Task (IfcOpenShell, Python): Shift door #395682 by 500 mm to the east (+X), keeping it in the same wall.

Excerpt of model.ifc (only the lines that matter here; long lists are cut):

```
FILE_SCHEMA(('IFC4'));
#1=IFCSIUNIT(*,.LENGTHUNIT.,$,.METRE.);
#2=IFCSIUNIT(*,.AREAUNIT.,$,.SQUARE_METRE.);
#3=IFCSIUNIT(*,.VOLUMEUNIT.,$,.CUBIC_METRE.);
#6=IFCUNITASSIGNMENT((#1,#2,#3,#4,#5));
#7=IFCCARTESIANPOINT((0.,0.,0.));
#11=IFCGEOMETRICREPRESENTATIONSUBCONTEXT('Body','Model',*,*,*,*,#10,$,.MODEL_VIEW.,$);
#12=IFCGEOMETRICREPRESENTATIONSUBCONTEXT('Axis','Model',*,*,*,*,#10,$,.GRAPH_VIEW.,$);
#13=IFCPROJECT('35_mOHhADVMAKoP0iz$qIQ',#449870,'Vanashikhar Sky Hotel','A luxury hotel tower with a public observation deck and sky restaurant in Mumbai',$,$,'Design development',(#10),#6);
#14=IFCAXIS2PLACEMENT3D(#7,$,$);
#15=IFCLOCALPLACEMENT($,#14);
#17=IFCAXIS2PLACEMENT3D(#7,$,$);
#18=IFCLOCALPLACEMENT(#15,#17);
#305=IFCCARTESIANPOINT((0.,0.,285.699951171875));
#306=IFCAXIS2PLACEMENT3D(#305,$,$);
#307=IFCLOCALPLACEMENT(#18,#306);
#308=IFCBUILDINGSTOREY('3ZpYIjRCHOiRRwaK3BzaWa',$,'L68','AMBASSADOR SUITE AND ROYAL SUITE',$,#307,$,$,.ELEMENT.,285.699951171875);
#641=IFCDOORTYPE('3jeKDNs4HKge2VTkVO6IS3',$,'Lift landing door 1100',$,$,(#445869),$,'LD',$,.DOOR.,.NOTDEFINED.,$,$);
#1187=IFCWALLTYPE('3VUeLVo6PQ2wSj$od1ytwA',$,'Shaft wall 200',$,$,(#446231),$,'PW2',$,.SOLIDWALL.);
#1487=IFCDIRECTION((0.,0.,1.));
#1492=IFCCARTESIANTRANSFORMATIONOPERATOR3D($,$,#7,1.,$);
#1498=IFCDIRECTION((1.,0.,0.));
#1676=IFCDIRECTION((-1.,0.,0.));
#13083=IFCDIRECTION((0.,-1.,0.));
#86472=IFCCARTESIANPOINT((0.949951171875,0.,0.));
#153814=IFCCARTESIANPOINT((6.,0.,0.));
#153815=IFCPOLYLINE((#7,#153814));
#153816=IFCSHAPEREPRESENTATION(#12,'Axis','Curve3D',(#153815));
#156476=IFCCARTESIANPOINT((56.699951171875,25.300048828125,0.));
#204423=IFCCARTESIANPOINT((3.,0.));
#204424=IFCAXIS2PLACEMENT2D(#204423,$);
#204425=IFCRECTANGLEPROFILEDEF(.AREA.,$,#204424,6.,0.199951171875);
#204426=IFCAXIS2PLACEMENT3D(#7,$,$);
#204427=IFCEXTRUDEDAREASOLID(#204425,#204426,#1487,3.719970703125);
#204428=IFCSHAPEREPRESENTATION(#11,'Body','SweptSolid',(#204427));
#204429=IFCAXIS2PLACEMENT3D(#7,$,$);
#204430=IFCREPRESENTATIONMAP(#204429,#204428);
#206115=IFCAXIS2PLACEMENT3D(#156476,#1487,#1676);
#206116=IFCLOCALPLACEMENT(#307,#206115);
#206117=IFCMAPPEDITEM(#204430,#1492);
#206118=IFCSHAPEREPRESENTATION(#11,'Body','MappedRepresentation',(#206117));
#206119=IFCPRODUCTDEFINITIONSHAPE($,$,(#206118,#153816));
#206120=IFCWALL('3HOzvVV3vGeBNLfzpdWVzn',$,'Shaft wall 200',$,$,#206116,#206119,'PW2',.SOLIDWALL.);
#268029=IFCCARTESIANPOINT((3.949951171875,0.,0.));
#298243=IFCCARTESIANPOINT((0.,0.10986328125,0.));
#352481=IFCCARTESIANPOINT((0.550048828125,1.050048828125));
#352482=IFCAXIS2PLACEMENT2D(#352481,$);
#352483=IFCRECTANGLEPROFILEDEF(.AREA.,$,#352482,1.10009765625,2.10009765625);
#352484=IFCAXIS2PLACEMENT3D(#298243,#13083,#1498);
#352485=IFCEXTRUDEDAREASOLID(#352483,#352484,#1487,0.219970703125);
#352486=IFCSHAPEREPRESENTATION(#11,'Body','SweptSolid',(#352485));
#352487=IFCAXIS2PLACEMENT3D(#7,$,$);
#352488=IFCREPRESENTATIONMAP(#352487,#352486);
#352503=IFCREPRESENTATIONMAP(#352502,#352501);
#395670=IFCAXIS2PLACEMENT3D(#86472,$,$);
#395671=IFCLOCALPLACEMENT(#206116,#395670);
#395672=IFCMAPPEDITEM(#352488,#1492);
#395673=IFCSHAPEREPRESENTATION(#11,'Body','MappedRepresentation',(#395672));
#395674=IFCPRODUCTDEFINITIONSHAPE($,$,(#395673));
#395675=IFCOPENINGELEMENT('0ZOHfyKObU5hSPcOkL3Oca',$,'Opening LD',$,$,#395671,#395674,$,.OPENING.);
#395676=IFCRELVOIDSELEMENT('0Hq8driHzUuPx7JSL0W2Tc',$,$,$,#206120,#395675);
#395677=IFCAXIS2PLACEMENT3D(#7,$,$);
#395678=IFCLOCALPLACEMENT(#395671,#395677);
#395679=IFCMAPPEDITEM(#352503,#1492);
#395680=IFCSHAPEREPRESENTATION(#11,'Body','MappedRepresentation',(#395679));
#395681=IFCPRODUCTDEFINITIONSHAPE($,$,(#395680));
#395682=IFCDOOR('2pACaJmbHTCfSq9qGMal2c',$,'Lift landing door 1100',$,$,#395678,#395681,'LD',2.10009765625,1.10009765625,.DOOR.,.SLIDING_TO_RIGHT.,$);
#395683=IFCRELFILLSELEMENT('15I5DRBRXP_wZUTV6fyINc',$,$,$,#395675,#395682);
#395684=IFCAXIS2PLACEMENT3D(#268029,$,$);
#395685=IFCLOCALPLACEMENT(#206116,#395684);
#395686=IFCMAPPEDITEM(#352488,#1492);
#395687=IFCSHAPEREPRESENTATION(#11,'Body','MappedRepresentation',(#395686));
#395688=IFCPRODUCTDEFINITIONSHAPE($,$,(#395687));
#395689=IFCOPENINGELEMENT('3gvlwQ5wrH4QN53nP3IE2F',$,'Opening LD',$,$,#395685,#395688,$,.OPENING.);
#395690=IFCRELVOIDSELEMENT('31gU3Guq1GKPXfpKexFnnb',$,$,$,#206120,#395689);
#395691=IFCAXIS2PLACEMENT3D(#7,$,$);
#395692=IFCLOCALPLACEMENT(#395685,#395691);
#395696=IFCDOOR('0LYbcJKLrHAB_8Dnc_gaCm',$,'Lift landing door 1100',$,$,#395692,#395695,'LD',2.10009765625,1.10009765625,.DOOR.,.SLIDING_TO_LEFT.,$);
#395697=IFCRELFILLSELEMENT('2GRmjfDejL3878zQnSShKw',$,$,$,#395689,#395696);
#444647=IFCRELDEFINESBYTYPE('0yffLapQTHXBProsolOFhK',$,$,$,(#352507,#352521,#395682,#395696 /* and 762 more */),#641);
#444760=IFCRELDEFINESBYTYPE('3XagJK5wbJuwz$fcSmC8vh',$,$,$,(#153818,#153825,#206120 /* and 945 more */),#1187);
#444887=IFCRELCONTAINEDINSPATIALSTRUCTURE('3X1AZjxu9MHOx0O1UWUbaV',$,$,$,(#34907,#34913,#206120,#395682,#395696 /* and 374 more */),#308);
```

```python
import ifcopenshell
import ifcopenshell.api.geometry
import ifcopenshell.util.placement
import ifcopenshell.util.unit

model = ifcopenshell.open("model.ifc")
unit_scale = ifcopenshell.util.unit.calculate_unit_scale(model)

door = model.by_guid("2pACaJmbHTCfSq9qGMal2c")
opening = door.FillsVoids[0].RelatingOpeningElement
wall = opening.VoidsElements[0].RelatingBuildingElement

wall_matrix = ifcopenshell.util.placement.get_local_placement(wall.ObjectPlacement)
shift = wall_matrix[:3, 0] * -0.5 / unit_scale
before = ifcopenshell.util.placement.get_local_placement(door.ObjectPlacement)[:3, 3].copy()

# The door is placed relative to its opening, so it follows when the opening moves.
matrix = ifcopenshell.util.placement.get_local_placement(opening.ObjectPlacement)
matrix[:3, 3] += shift
ifcopenshell.api.geometry.edit_object_placement(
    model, product=opening, matrix=matrix, is_si=False, should_transform_children=True
)

after = ifcopenshell.util.placement.get_local_placement(door.ObjectPlacement)[:3, 3]
print("door moved by", (after - before).round(3) + 0.0)

model.write("model_v2.ifc")
```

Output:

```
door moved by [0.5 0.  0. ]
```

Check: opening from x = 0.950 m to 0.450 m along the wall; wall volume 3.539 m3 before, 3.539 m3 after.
